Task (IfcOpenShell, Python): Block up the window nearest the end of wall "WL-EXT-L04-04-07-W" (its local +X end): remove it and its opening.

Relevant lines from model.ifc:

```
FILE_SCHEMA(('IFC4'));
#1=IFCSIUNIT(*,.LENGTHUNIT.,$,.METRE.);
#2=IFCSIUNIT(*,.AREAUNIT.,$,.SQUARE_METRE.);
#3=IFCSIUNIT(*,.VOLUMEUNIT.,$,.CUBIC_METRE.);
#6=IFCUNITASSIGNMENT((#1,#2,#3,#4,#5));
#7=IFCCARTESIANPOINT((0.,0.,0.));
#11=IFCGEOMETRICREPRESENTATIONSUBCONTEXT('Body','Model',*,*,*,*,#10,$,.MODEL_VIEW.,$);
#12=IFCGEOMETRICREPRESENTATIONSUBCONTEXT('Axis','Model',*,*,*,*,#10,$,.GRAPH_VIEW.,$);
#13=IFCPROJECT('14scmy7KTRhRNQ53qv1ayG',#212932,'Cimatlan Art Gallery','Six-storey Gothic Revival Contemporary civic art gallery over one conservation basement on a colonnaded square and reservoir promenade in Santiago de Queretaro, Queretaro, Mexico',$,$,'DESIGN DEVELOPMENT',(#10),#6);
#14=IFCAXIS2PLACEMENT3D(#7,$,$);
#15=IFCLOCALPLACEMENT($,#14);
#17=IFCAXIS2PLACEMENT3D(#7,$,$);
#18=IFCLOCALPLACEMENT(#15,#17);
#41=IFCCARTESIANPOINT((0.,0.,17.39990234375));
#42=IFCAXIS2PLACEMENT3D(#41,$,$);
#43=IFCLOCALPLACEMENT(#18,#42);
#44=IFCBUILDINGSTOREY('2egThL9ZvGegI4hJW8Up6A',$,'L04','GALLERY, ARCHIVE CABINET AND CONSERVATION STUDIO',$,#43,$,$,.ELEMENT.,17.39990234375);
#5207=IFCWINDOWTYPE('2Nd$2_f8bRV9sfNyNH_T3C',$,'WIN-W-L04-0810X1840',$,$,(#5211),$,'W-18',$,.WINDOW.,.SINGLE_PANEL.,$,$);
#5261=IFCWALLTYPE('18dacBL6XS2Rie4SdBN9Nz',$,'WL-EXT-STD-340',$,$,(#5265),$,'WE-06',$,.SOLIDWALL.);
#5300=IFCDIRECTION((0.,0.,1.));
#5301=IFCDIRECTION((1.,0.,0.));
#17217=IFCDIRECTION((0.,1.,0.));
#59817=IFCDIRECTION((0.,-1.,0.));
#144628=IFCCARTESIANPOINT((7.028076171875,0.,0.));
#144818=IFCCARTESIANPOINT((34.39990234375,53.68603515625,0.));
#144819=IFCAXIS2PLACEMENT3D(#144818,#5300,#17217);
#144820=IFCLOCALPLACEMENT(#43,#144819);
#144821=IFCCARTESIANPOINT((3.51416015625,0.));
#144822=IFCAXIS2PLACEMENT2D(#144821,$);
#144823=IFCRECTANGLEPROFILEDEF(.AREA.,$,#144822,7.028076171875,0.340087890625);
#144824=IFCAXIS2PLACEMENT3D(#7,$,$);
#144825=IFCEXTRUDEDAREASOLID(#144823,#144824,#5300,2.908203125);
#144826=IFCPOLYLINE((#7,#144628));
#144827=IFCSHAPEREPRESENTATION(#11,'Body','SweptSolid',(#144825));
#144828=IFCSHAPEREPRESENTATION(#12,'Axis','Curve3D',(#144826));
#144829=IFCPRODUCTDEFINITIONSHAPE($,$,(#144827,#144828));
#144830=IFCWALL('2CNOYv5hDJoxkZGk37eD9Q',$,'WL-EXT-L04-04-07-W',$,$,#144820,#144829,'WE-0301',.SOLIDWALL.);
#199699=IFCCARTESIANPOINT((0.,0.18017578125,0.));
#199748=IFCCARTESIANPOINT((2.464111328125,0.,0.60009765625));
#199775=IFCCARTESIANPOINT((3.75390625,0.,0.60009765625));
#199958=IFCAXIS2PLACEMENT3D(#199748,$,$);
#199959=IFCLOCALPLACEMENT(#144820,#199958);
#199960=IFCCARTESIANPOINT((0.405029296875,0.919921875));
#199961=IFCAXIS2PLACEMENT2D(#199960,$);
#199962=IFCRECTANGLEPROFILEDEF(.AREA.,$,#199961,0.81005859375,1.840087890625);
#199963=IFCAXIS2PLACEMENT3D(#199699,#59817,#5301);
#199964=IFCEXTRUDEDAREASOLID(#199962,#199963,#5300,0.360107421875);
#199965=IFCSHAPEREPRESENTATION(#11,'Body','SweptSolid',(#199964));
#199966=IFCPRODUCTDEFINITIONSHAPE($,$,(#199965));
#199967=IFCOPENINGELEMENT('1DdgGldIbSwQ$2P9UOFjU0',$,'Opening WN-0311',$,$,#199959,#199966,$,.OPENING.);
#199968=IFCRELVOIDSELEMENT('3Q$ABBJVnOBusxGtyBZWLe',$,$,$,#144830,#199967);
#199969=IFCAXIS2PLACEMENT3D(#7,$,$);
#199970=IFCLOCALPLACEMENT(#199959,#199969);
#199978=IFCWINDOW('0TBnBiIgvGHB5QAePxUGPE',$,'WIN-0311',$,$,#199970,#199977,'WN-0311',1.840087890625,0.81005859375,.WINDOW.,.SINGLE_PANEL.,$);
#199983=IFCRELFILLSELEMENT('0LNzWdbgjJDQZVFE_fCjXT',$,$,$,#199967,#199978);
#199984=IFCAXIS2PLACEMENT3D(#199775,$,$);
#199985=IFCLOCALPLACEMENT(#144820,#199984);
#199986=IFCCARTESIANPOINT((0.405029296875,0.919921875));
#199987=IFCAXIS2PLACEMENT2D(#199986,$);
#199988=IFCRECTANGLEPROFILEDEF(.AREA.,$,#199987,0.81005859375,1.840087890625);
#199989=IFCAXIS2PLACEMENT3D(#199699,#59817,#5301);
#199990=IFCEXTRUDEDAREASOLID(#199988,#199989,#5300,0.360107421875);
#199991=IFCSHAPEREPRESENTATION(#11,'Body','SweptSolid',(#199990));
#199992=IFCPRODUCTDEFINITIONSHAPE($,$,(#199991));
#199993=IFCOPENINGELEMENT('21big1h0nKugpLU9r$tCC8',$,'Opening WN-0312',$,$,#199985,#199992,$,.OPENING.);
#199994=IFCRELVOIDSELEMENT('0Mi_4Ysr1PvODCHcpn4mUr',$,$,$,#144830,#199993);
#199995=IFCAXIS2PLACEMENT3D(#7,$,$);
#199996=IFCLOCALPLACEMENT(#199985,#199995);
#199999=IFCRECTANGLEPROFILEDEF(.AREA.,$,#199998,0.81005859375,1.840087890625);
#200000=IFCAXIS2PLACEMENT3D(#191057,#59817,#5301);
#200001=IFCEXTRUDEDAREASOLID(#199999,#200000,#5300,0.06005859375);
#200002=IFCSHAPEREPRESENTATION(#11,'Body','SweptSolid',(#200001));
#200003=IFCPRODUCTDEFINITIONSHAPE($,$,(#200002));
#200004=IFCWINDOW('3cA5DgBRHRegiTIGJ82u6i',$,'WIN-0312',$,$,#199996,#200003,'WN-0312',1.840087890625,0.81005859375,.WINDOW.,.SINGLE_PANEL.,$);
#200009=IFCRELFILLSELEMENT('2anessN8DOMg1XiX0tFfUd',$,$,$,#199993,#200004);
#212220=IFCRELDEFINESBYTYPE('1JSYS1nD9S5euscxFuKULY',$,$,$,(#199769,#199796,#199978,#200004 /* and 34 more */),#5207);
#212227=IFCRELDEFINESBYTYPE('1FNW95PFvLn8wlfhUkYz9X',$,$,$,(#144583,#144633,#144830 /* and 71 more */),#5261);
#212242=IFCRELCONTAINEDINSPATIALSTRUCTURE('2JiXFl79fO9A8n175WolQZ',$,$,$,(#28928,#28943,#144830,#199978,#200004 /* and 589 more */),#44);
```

```python
import ifcopenshell
import ifcopenshell.api.feature
import ifcopenshell.api.root
import ifcopenshell.geom
import ifcopenshell.util.shape

model = ifcopenshell.open("model.ifc")
settings = ifcopenshell.geom.settings()


def volume(element):
    """Net volume in cubic metres, openings subtracted."""
    shape = ifcopenshell.geom.create_shape(settings, element)
    return ifcopenshell.util.shape.get_volume(shape.geometry)


window = model.by_id(200004)
opening = window.FillsVoids[0].RelatingOpeningElement
wall = opening.VoidsElements[0].RelatingBuildingElement
before = volume(wall)

ifcopenshell.api.root.remove_product(model, product=window)
ifcopenshell.api.feature.remove_feature(model, feature=opening)

after = volume(wall)

print(f"wall volume {before:.3f} -> {after:.3f} m3")

model.write("model-out.ifc")
```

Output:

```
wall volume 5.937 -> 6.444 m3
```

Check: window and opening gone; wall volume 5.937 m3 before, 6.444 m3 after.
